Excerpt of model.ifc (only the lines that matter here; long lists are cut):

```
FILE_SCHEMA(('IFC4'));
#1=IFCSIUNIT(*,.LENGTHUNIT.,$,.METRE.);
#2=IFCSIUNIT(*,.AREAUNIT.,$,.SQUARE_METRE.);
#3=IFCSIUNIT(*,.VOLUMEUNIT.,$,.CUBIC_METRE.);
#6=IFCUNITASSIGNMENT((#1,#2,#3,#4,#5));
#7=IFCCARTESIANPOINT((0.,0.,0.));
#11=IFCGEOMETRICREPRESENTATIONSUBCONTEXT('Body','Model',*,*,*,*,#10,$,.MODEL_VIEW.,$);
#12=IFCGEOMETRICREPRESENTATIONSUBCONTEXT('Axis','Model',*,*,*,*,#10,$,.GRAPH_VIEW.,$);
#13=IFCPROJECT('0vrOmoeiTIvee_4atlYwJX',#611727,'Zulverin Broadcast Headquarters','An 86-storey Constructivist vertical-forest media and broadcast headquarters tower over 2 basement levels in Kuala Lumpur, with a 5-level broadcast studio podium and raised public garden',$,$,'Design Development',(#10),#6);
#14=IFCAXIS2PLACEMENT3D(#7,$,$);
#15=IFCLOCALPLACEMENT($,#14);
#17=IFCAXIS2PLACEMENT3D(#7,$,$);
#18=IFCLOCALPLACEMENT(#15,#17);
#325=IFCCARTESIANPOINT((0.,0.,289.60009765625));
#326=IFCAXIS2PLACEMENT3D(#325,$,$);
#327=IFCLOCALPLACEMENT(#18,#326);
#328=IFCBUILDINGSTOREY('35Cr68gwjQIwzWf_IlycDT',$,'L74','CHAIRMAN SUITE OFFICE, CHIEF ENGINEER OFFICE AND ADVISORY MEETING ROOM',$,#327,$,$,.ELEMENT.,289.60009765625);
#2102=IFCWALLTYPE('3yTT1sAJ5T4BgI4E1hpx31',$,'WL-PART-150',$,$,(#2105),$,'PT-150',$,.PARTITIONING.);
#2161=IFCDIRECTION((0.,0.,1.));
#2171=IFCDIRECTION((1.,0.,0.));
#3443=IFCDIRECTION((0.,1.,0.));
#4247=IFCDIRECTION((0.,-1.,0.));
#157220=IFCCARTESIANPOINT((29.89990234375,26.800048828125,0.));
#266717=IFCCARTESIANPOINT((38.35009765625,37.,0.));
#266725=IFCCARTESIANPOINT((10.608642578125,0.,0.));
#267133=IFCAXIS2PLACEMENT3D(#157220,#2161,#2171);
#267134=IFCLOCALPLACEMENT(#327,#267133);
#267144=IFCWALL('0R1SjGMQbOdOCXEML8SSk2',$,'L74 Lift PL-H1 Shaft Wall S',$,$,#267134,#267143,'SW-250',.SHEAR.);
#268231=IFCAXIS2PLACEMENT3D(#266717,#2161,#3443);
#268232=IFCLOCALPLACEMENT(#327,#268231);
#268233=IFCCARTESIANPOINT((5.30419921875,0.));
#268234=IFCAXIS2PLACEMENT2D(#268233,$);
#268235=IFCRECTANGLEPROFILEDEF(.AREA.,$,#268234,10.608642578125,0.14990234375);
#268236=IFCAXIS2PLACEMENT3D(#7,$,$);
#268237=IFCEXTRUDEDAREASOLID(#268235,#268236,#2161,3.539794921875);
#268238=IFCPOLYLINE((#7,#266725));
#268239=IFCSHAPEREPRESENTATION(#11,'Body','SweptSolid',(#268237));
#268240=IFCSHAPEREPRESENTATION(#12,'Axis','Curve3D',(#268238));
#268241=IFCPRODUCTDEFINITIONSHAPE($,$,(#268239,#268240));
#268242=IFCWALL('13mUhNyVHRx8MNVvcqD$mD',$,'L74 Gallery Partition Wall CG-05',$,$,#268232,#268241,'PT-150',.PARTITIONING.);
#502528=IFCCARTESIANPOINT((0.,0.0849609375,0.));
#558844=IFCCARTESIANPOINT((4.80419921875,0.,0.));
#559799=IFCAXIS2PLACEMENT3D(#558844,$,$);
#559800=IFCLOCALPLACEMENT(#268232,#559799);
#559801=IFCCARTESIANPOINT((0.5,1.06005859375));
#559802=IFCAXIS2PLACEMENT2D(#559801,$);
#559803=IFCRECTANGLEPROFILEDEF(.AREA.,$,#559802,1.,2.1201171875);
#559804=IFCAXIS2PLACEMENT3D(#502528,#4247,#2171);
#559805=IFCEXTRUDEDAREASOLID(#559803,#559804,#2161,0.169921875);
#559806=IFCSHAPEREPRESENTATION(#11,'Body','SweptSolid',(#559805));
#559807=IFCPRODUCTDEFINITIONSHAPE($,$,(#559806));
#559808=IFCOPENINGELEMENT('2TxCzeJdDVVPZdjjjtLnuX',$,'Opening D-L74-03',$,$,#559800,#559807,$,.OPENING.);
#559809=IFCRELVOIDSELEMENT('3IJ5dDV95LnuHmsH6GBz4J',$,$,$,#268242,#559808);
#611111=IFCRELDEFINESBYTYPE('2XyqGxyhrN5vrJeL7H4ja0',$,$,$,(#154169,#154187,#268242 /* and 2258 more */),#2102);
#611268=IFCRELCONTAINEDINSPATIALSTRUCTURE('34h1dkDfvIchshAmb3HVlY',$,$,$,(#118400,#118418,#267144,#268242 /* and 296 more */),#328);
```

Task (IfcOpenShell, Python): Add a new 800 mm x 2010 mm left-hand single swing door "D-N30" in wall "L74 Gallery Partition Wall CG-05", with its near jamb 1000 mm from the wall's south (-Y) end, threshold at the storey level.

```python
import numpy as np
import ifcopenshell
import ifcopenshell.api.feature
import ifcopenshell.api.geometry
import ifcopenshell.api.root
import ifcopenshell.api.spatial
import ifcopenshell.geom
import ifcopenshell.util.element
import ifcopenshell.util.placement
import ifcopenshell.util.representation
import ifcopenshell.util.shape
import ifcopenshell.util.unit

model = ifcopenshell.open("model.ifc")
unit_scale = ifcopenshell.util.unit.calculate_unit_scale(model)
settings = ifcopenshell.geom.settings()


def volume(element):
    """Net volume in cubic metres, openings subtracted."""
    shape = ifcopenshell.geom.create_shape(settings, element)
    return ifcopenshell.util.shape.get_volume(shape.geometry)


wall = model.by_guid("13mUhNyVHRx8MNVvcqD$mD")
storey = ifcopenshell.util.element.get_container(wall, ifc_class="IfcBuildingStorey")
context = ifcopenshell.util.representation.get_context(model, "Model", "Body", "MODEL_VIEW")
before = volume(wall)

width, height, from_end, sill = 0.8, 2.01, 1, 0.0  # metres

# The wall runs along its own X axis, and the end named is its -X end.
wall_shape = ifcopenshell.geom.create_shape(settings, wall)
x, y, z = ifcopenshell.util.shape.get_vertices(wall_shape.geometry).T
start = x.min() + from_end
face, thickness = float(y.min()), float(y.max() - y.min())
wall_matrix = ifcopenshell.util.placement.get_local_placement(wall.ObjectPlacement)
level = ifcopenshell.util.placement.get_local_placement(storey.ObjectPlacement)[2, 3]


def in_wall(x, y):
    """Placement at x, y metres in the wall's axes, at sill height."""
    matrix = wall_matrix.copy()
    matrix[:, 3] = wall_matrix @ np.array([x / unit_scale, y / unit_scale, 0.0, 1.0])
    matrix[2, 3] = level + sill / unit_scale
    return matrix


# Opening: a box that overshoots both wall faces by 50 mm.
opening = ifcopenshell.api.root.create_entity(model, ifc_class="IfcOpeningElement", predefined_type="OPENING")
box = ifcopenshell.api.geometry.add_wall_representation(
    model, context=context, length=width, height=height, thickness=thickness + 0.1
)
ifcopenshell.api.geometry.assign_representation(model, product=opening, representation=box)
ifcopenshell.api.geometry.edit_object_placement(model, product=opening, matrix=in_wall(start, face - 0.05), is_si=False)
ifcopenshell.api.feature.add_feature(model, feature=opening, element=wall)

door = ifcopenshell.api.root.create_entity(model, ifc_class="IfcDoor", name="D-N30", predefined_type="DOOR")
door.OverallWidth, door.OverallHeight = width / unit_scale, height / unit_scale
door.OperationType = "SINGLE_SWING_LEFT"
body = ifcopenshell.api.geometry.add_door_representation(
    model,
    context=context,
    overall_width=door.OverallWidth,
    overall_height=door.OverallHeight,
    operation_type="SINGLE_SWING_LEFT",
    lining_properties={"LiningDepth": thickness / unit_scale, "ThresholdDepth": thickness / unit_scale},
)
ifcopenshell.api.geometry.assign_representation(model, product=door, representation=body)
ifcopenshell.api.spatial.assign_container(model, products=[door], relating_structure=storey)
ifcopenshell.api.feature.add_filling(model, opening=opening, element=door)

# The lining spans the wall, so the door starts at the wall face.
ifcopenshell.api.geometry.edit_object_placement(model, product=door, matrix=in_wall(start, face), is_si=False)

after = volume(wall)

print(f"wall volume {before:.3f} -> {after:.3f} m3")

model.write("model_updated.ifc")
```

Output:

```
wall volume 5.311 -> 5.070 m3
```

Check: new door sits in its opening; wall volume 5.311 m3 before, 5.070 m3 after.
